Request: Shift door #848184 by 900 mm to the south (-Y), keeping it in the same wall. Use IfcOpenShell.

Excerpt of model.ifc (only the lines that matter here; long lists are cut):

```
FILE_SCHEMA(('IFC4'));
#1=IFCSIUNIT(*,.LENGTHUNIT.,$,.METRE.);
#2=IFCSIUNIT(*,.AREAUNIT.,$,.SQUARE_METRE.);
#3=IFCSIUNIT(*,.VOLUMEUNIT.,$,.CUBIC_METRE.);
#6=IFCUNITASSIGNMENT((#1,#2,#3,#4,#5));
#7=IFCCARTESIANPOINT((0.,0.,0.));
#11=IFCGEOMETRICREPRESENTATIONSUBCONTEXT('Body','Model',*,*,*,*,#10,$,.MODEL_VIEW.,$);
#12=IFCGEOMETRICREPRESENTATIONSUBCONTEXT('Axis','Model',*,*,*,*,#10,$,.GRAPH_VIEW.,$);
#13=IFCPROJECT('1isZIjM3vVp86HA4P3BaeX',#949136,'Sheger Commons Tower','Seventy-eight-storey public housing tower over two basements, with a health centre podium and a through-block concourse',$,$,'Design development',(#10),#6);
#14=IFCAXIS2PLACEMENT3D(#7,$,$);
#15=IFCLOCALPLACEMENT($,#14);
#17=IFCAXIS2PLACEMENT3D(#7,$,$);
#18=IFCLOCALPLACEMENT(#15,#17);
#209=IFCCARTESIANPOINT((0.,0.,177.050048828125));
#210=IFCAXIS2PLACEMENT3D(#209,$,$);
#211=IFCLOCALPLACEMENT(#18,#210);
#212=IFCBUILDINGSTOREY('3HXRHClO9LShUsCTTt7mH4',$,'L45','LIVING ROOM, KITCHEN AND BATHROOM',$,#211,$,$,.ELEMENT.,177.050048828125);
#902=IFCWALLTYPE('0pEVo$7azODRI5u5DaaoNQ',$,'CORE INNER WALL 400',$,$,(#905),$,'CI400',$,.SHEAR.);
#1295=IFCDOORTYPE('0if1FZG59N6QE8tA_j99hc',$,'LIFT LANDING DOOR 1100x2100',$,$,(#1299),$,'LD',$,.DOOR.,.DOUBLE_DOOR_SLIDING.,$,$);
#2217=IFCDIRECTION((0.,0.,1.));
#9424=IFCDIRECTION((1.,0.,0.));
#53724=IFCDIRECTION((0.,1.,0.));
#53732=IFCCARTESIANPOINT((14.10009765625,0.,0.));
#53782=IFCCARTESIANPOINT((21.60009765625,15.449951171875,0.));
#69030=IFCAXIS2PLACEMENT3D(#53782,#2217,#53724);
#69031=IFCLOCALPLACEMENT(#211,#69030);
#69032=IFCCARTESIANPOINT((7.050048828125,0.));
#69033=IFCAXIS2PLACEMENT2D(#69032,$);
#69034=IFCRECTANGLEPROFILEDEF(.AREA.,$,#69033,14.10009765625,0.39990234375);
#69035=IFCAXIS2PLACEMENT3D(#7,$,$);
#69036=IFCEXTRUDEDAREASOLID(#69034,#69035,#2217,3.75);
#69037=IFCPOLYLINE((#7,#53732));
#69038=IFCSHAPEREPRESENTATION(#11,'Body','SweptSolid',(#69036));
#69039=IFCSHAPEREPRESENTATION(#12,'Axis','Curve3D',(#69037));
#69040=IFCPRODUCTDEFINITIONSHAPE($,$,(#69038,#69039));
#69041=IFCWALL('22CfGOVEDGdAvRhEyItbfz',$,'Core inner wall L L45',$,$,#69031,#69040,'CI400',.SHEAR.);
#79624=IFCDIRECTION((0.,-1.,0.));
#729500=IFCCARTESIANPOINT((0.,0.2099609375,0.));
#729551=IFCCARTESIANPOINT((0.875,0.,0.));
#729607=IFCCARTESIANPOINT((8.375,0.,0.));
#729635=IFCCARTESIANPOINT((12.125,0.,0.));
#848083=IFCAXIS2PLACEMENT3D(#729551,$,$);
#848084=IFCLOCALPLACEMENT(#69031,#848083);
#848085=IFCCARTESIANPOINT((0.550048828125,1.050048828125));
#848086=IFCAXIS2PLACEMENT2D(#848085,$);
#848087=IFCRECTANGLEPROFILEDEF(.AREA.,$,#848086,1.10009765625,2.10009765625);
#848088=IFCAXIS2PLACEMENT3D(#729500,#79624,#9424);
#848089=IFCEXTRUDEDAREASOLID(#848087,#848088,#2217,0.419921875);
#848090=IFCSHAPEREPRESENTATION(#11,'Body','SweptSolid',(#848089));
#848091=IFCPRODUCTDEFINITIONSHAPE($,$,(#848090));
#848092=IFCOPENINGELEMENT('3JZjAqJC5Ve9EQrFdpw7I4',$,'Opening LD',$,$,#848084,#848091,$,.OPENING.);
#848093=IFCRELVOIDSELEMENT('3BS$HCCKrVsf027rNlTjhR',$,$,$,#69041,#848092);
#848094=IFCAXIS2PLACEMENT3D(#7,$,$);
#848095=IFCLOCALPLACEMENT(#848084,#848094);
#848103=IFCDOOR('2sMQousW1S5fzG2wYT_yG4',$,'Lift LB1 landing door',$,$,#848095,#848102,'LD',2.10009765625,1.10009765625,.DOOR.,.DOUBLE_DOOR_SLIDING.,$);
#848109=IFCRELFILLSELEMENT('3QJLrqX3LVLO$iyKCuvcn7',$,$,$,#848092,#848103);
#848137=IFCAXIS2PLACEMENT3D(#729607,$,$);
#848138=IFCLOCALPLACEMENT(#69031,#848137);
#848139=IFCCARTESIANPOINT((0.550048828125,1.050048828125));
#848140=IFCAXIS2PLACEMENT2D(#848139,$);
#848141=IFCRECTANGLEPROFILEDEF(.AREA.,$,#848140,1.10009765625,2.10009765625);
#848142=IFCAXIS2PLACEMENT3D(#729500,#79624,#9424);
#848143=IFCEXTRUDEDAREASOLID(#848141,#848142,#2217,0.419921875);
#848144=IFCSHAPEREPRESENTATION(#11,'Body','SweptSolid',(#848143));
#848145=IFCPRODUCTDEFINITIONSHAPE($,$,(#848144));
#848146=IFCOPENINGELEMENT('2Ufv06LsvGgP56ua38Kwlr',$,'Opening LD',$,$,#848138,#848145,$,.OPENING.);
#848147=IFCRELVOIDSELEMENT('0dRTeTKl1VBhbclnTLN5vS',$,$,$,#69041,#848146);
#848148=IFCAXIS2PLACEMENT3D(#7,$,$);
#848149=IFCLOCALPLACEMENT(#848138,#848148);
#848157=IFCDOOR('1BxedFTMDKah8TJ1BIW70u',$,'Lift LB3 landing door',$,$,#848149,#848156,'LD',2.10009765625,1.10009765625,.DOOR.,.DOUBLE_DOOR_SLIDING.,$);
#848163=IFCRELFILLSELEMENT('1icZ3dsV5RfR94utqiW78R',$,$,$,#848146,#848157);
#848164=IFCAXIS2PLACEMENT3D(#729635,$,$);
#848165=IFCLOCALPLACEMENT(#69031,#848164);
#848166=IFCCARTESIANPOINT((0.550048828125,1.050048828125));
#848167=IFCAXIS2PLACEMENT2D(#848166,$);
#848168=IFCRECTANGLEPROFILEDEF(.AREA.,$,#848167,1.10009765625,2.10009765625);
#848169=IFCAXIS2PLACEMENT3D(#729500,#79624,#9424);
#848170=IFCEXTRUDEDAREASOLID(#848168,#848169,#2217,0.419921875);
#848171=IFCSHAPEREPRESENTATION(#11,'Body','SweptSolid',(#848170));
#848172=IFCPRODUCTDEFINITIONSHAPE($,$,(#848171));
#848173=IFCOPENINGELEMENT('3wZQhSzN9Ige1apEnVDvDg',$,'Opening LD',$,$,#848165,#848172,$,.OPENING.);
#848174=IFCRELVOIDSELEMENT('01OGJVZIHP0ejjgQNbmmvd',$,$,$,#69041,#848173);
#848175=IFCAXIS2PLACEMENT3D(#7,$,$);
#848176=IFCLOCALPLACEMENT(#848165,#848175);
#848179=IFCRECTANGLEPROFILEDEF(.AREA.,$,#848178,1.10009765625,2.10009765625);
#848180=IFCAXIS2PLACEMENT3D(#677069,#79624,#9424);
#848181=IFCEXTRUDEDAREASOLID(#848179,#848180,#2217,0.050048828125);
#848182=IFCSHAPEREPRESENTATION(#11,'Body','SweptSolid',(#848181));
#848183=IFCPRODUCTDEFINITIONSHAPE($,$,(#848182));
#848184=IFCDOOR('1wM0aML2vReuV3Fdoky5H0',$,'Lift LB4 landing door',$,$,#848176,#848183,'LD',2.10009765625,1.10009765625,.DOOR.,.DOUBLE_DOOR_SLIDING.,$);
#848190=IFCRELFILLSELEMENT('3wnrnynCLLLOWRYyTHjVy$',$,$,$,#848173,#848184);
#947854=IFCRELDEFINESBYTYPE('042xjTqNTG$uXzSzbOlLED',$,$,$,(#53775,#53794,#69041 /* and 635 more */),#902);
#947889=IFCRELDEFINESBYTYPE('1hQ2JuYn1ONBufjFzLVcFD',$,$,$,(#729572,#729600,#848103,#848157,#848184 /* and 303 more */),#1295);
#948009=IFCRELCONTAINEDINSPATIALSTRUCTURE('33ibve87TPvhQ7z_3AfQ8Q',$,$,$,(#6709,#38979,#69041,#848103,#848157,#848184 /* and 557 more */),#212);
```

```python
import ifcopenshell
import ifcopenshell.api.geometry
import ifcopenshell.util.placement
import ifcopenshell.util.unit

model = ifcopenshell.open("model.ifc")
unit_scale = ifcopenshell.util.unit.calculate_unit_scale(model)

door = model.by_guid("1wM0aML2vReuV3Fdoky5H0")
opening = door.FillsVoids[0].RelatingOpeningElement
wall = opening.VoidsElements[0].RelatingBuildingElement

wall_matrix = ifcopenshell.util.placement.get_local_placement(wall.ObjectPlacement)
shift = wall_matrix[:3, 0] * -0.9 / unit_scale
before = ifcopenshell.util.placement.get_local_placement(door.ObjectPlacement)[:3, 3].copy()

# The door is placed relative to its opening, so it follows when the opening moves.
matrix = ifcopenshell.util.placement.get_local_placement(opening.ObjectPlacement)
matrix[:3, 3] += shift
ifcopenshell.api.geometry.edit_object_placement(
    model, product=opening, matrix=matrix, is_si=False, should_transform_children=True
)

after = ifcopenshell.util.placement.get_local_placement(door.ObjectPlacement)[:3, 3]
print("door moved by", (after - before).round(3) + 0.0)

model.write("model_edited.ifc")
```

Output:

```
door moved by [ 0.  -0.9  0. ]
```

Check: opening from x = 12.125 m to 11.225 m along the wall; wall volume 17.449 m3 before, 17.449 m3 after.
